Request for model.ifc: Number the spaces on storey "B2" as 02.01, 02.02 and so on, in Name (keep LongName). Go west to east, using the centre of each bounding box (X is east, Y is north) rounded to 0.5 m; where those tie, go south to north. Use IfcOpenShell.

First a look at what the model holds.

```python
import ifcopenshell
import ifcopenshell.util.element
import ifcopenshell.util.placement

model = ifcopenshell.open("model.ifc")
print(model.schema)
storey = next(s for s in model.by_type("IfcBuildingStorey") if s.Name == "B2")
spaces = [e for e in ifcopenshell.util.element.get_decomposition(storey) if e.is_a("IfcSpace")]
for e in sorted(spaces, key=lambda e: e.id()):
    origin = ifcopenshell.util.placement.get_local_placement(e.ObjectPlacement)[:3, 3]
    print(e.id(), e.Name, e.LongName, origin.round(2) + 0.0, sep=" | ")
```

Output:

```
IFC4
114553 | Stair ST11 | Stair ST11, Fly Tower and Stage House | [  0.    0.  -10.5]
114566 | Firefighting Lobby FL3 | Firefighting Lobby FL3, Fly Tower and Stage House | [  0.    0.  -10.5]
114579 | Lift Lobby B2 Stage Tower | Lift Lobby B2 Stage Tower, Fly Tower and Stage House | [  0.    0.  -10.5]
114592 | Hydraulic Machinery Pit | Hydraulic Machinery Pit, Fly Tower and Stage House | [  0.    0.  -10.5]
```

```python
import ifcopenshell
import ifcopenshell.geom
import ifcopenshell.util.element
import ifcopenshell.util.shape

model = ifcopenshell.open("model.ifc")
settings = ifcopenshell.geom.settings()
settings.set("use-world-coords", True)


def centre(element):
    shape = ifcopenshell.geom.create_shape(settings, element)
    return ifcopenshell.util.shape.get_bbox_centroid(shape.geometry)


storey = next(s for s in model.by_type("IfcBuildingStorey") if s.Name == "B2")
spaces = [e for e in ifcopenshell.util.element.get_decomposition(storey) if e.is_a("IfcSpace")]

# Insertion points can sit at a corner or the storey origin, so sort by the geometry (in metres).
centres = {e: centre(e) for e in spaces}
spaces.sort(key=lambda e: (round(centres[e][0] / 0.5), centres[e][1]))

for i, e in enumerate(spaces, start=1):
    number = f"02.{i:02d}"
    e.Name = number
    print(e.id(), number)

model.write("model_v2.ifc")
```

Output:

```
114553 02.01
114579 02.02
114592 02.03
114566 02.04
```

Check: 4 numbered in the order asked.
